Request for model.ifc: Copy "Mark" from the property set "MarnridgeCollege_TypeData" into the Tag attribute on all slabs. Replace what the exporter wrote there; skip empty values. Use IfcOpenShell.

First a look at what the model holds.

```python
import ifcopenshell
import ifcopenshell.util.element

model = ifcopenshell.open("model.ifc")
print(model.schema)
slabs = model.by_type("IfcSlab")
print(len(slabs), "slabs")
for e in slabs[:8]:
    source = ifcopenshell.util.element.get_pset(e, "MarnridgeCollege_TypeData", "Mark")
    target = e.Tag
    print(e.id(), repr(source), repr(target), sep=" | ")
```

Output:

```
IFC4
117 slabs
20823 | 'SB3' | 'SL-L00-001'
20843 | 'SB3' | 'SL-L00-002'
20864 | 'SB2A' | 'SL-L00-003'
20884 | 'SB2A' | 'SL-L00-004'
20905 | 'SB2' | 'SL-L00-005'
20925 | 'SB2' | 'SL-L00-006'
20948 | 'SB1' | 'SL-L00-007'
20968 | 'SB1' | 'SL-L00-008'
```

```python
import ifcopenshell
import ifcopenshell.util.element

model = ifcopenshell.open("model.ifc")

count = 0
for e in model.by_type("IfcSlab"):
    value = ifcopenshell.util.element.get_pset(e, "MarnridgeCollege_TypeData", "Mark")
    current = e.Tag
    if not value or not value.strip() or current == value:
        continue
    e.Tag = value
    count += 1

print(count, "slabs updated")

model.write("model-out.ifc")
```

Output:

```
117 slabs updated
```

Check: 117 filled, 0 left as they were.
